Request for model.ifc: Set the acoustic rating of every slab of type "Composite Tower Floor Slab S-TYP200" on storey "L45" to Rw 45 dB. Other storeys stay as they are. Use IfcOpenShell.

First a look at what the model holds.

```python
import ifcopenshell
import ifcopenshell.util.element

model = ifcopenshell.open("model.ifc")
print(model.schema)
storey = next(s for s in model.by_type("IfcBuildingStorey") if s.Name == "L45")
slabs = [e for e in ifcopenshell.util.element.get_decomposition(storey) if e.is_a("IfcSlab")]
seen = {}
for e in slabs:
    element_type = ifcopenshell.util.element.get_type(e)
    key = (element_type.Name if element_type != e and element_type else None, ifcopenshell.util.element.get_pset(e, "Pset_SlabCommon", "AcousticRating"))
    seen[key] = seen.get(key, 0) + 1
for (name, value), count in sorted(seen.items(), key=str):
    print(count, "x", name, "|", value)
```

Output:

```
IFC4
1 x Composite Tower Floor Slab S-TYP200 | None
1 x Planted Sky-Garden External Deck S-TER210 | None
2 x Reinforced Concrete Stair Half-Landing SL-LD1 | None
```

```python
import ifcopenshell
import ifcopenshell.api.pset
import ifcopenshell.util.element

model = ifcopenshell.open("model.ifc")

storey = next(s for s in model.by_type("IfcBuildingStorey") if s.Name == "L45")
slabs = [e for e in ifcopenshell.util.element.get_decomposition(storey) if e.is_a("IfcSlab")]

count = 0
for e in slabs:
    element_type = ifcopenshell.util.element.get_type(e)
    if element_type in (None, e) or element_type.Name != "Composite Tower Floor Slab S-TYP200":
        continue
    found = ifcopenshell.util.element.get_pset(e, "Pset_SlabCommon", should_inherit=False)
    if found:
        pset = model.by_id(found["id"])
        if len(ifcopenshell.util.element.get_elements_by_pset(pset)) > 1:
            pset = ifcopenshell.api.pset.unshare_pset(model, products=[e], pset=pset)[0]
    else:
        pset = ifcopenshell.api.pset.add_pset(model, product=e, name="Pset_SlabCommon")
    ifcopenshell.api.pset.edit_pset(model, pset=pset, properties={"AcousticRating": "Rw 45 dB"})
    count += 1

print(count, "slabs updated")

model.write("model_updated.ifc")
```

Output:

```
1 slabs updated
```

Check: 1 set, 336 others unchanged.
